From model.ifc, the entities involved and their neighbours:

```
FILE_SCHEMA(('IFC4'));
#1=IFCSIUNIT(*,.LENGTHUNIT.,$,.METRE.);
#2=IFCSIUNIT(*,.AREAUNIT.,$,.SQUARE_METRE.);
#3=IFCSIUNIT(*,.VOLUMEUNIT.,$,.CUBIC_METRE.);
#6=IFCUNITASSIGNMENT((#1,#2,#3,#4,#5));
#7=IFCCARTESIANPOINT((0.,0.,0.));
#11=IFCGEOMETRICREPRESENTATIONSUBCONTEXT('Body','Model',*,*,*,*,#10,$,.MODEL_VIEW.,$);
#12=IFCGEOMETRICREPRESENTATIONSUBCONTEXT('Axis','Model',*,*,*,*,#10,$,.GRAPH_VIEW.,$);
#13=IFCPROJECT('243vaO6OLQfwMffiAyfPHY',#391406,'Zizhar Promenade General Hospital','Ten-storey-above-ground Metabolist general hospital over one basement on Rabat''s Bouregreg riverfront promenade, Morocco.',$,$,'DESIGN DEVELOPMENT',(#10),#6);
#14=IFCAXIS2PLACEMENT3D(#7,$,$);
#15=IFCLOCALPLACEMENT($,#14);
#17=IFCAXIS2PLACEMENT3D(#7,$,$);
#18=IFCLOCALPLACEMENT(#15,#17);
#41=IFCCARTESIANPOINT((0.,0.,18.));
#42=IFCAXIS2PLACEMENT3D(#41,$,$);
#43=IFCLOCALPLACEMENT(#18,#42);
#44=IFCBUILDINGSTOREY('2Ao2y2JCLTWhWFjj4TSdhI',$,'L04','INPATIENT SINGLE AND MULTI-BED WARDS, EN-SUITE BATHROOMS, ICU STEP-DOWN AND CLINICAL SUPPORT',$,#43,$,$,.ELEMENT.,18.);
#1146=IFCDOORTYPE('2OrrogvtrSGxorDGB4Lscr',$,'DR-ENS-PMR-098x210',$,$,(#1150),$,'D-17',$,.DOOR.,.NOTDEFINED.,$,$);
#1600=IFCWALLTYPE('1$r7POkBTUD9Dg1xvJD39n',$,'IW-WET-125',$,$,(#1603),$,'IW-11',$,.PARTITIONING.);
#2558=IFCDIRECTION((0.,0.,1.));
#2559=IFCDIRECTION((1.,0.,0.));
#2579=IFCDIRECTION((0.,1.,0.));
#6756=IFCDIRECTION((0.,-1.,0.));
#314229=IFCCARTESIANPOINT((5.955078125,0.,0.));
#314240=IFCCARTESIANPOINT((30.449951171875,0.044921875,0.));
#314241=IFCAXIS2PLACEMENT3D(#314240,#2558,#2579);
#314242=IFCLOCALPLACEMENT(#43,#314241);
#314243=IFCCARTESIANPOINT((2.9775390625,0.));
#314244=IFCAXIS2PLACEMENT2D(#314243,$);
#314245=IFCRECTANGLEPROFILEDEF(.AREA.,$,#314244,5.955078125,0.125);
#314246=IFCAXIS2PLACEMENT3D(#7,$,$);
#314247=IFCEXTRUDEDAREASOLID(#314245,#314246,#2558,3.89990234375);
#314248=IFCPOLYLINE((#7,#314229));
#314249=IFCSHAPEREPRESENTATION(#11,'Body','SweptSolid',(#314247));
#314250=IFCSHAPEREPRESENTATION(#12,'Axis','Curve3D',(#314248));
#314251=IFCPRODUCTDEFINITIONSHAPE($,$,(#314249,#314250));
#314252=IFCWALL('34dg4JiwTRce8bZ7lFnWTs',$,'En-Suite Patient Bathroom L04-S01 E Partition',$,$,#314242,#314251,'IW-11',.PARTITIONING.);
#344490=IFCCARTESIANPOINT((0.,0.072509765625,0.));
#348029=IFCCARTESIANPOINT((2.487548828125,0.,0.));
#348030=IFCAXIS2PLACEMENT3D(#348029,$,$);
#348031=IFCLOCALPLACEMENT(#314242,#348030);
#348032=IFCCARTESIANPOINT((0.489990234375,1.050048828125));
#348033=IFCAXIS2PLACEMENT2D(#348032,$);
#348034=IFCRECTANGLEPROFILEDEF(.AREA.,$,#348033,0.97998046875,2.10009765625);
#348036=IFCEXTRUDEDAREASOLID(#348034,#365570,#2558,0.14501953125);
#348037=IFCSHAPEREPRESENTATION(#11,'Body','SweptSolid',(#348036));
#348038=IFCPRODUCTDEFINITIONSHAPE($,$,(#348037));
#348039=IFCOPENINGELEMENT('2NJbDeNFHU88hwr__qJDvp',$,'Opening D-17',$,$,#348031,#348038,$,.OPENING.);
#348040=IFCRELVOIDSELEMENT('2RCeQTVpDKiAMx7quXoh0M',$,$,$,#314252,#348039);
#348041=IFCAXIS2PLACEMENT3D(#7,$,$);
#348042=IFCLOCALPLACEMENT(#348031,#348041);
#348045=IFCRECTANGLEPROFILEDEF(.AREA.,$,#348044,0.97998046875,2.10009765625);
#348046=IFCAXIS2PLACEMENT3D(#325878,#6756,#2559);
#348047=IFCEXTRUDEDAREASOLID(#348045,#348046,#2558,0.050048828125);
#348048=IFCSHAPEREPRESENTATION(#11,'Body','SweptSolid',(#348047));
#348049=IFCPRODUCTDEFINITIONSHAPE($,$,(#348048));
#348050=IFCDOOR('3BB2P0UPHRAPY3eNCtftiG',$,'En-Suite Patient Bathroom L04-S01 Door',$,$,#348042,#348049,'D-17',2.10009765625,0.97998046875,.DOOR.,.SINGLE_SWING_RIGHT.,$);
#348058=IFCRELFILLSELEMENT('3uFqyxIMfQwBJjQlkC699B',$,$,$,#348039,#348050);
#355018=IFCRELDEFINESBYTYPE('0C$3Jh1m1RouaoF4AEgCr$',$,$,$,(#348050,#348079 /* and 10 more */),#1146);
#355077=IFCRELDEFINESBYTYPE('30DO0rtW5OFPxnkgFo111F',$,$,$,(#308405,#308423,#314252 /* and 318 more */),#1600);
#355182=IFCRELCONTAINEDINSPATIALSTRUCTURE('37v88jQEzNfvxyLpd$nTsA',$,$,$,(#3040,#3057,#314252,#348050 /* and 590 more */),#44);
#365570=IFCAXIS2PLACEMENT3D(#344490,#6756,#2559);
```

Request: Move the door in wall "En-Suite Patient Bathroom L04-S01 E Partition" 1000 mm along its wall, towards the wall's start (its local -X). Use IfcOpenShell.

```python
import ifcopenshell
import ifcopenshell.api.geometry
import ifcopenshell.util.placement
import ifcopenshell.util.unit

model = ifcopenshell.open("model.ifc")
unit_scale = ifcopenshell.util.unit.calculate_unit_scale(model)

door = model.by_guid("3BB2P0UPHRAPY3eNCtftiG")
opening = door.FillsVoids[0].RelatingOpeningElement
wall = opening.VoidsElements[0].RelatingBuildingElement

wall_matrix = ifcopenshell.util.placement.get_local_placement(wall.ObjectPlacement)
shift = wall_matrix[:3, 0] * -1 / unit_scale
before = ifcopenshell.util.placement.get_local_placement(door.ObjectPlacement)[:3, 3].copy()

# The door is placed relative to its opening, so it follows when the opening moves.
matrix = ifcopenshell.util.placement.get_local_placement(opening.ObjectPlacement)
matrix[:3, 3] += shift
ifcopenshell.api.geometry.edit_object_placement(
    model, product=opening, matrix=matrix, is_si=False, should_transform_children=True
)

after = ifcopenshell.util.placement.get_local_placement(door.ObjectPlacement)[:3, 3]
print("door moved by", (after - before).round(3) + 0.0)

model.write("model_updated.ifc")
```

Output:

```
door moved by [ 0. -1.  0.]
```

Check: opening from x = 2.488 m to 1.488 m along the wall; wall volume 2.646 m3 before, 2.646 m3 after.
